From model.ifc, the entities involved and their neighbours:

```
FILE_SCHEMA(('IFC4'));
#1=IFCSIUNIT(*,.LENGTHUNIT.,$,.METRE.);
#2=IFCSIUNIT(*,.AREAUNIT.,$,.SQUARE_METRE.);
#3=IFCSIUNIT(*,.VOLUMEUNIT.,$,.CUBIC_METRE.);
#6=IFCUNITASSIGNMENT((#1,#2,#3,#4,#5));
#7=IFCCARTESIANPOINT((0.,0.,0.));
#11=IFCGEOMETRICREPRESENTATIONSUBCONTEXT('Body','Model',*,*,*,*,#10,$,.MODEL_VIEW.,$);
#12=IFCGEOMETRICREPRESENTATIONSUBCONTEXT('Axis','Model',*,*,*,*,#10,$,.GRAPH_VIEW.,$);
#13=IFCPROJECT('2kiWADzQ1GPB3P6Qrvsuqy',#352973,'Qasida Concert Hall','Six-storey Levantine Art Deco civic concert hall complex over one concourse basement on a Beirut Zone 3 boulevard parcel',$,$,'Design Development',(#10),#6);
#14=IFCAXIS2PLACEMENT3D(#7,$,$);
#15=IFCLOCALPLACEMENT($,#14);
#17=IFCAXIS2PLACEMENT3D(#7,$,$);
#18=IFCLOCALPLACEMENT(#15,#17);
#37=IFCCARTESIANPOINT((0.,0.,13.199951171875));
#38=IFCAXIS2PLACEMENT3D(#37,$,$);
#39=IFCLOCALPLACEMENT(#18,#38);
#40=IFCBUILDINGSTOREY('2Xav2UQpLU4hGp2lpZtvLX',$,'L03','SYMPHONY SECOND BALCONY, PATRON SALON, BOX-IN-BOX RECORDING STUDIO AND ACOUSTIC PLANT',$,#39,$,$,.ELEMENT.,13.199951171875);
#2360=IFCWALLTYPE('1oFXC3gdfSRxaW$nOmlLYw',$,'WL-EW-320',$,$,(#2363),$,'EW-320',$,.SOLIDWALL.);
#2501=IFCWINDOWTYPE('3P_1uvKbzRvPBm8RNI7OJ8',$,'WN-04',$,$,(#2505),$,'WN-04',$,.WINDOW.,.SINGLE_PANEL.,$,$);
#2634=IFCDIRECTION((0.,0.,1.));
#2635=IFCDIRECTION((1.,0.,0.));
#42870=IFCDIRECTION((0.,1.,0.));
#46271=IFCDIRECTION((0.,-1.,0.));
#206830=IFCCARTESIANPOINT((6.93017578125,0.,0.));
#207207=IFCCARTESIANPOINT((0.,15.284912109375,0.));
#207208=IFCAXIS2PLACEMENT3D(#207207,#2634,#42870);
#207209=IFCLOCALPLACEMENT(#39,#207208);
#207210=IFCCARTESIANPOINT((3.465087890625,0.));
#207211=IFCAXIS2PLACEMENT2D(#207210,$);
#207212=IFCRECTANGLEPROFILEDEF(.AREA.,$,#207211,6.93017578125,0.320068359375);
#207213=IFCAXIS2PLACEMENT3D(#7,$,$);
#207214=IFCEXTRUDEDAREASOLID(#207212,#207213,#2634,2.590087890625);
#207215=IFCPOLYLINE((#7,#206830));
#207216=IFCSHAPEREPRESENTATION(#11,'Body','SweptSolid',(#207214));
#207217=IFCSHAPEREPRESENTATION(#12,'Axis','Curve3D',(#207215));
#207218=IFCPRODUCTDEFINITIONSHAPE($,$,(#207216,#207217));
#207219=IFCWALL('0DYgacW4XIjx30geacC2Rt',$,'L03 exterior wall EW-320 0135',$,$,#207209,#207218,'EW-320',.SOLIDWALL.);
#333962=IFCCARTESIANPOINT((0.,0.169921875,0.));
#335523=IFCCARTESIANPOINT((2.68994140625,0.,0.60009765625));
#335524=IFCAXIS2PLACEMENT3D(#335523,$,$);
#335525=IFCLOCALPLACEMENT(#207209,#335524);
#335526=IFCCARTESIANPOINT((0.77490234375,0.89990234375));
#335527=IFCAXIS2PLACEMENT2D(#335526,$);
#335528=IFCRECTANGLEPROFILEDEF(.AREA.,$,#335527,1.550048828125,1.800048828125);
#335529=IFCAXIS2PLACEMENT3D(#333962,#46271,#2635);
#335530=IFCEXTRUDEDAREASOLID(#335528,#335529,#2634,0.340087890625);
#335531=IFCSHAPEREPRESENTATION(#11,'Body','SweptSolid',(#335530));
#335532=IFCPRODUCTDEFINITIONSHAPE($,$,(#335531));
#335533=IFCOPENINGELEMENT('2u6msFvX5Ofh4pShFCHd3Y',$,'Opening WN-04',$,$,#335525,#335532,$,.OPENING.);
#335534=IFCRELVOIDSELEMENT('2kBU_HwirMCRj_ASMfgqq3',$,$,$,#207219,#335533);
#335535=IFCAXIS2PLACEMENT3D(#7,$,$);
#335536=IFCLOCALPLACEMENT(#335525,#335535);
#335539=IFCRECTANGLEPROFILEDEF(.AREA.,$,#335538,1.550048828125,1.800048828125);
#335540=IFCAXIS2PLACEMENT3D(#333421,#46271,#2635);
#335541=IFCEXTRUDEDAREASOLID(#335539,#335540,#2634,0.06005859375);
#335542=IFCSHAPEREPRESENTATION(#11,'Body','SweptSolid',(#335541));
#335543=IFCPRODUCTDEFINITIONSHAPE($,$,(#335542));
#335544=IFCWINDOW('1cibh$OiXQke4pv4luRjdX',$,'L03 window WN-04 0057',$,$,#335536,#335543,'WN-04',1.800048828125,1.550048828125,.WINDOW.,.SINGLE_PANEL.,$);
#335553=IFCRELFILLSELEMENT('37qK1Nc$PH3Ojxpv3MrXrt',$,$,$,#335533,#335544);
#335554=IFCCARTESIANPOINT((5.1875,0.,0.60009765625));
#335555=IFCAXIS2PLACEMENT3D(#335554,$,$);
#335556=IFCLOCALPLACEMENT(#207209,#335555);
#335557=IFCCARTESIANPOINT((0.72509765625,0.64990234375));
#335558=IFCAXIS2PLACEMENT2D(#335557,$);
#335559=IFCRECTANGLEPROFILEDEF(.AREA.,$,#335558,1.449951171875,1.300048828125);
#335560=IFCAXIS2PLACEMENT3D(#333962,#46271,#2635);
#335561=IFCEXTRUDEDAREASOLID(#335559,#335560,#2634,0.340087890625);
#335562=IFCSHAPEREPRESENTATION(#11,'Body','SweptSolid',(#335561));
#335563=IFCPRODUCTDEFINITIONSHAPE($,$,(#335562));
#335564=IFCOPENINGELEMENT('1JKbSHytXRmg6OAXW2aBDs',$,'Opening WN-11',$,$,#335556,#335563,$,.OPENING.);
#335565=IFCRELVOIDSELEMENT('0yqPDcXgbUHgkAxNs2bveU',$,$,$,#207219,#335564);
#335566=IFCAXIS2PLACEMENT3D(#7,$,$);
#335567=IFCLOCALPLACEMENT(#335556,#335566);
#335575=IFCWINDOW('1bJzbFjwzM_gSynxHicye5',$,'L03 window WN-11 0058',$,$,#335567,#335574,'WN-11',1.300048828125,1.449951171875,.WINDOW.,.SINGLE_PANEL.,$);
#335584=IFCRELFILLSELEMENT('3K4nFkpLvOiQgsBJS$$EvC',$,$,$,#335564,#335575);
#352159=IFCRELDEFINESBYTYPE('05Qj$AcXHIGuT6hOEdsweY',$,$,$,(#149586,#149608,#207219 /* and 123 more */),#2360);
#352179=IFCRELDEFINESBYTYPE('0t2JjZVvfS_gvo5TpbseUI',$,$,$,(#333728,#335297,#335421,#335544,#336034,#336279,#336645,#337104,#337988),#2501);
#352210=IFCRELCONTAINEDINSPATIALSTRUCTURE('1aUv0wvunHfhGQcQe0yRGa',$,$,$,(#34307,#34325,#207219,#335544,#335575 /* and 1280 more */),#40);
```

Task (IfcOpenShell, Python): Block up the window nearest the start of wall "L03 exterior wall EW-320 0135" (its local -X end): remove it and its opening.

```python
import ifcopenshell
import ifcopenshell.api.feature
import ifcopenshell.api.root
import ifcopenshell.geom
import ifcopenshell.util.shape

model = ifcopenshell.open("model.ifc")
settings = ifcopenshell.geom.settings()


def volume(element):
    """Net volume in cubic metres, openings subtracted."""
    shape = ifcopenshell.geom.create_shape(settings, element)
    return ifcopenshell.util.shape.get_volume(shape.geometry)


window = model.by_guid("1cibh$OiXQke4pv4luRjdX")
opening = window.FillsVoids[0].RelatingOpeningElement
wall = opening.VoidsElements[0].RelatingBuildingElement
before = volume(wall)

ifcopenshell.api.root.remove_product(model, product=window)
ifcopenshell.api.feature.remove_feature(model, feature=opening)

after = volume(wall)

print(f"wall volume {before:.3f} -> {after:.3f} m3")

model.write("model_edited.ifc")
```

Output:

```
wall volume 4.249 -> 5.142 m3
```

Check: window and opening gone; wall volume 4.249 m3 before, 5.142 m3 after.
